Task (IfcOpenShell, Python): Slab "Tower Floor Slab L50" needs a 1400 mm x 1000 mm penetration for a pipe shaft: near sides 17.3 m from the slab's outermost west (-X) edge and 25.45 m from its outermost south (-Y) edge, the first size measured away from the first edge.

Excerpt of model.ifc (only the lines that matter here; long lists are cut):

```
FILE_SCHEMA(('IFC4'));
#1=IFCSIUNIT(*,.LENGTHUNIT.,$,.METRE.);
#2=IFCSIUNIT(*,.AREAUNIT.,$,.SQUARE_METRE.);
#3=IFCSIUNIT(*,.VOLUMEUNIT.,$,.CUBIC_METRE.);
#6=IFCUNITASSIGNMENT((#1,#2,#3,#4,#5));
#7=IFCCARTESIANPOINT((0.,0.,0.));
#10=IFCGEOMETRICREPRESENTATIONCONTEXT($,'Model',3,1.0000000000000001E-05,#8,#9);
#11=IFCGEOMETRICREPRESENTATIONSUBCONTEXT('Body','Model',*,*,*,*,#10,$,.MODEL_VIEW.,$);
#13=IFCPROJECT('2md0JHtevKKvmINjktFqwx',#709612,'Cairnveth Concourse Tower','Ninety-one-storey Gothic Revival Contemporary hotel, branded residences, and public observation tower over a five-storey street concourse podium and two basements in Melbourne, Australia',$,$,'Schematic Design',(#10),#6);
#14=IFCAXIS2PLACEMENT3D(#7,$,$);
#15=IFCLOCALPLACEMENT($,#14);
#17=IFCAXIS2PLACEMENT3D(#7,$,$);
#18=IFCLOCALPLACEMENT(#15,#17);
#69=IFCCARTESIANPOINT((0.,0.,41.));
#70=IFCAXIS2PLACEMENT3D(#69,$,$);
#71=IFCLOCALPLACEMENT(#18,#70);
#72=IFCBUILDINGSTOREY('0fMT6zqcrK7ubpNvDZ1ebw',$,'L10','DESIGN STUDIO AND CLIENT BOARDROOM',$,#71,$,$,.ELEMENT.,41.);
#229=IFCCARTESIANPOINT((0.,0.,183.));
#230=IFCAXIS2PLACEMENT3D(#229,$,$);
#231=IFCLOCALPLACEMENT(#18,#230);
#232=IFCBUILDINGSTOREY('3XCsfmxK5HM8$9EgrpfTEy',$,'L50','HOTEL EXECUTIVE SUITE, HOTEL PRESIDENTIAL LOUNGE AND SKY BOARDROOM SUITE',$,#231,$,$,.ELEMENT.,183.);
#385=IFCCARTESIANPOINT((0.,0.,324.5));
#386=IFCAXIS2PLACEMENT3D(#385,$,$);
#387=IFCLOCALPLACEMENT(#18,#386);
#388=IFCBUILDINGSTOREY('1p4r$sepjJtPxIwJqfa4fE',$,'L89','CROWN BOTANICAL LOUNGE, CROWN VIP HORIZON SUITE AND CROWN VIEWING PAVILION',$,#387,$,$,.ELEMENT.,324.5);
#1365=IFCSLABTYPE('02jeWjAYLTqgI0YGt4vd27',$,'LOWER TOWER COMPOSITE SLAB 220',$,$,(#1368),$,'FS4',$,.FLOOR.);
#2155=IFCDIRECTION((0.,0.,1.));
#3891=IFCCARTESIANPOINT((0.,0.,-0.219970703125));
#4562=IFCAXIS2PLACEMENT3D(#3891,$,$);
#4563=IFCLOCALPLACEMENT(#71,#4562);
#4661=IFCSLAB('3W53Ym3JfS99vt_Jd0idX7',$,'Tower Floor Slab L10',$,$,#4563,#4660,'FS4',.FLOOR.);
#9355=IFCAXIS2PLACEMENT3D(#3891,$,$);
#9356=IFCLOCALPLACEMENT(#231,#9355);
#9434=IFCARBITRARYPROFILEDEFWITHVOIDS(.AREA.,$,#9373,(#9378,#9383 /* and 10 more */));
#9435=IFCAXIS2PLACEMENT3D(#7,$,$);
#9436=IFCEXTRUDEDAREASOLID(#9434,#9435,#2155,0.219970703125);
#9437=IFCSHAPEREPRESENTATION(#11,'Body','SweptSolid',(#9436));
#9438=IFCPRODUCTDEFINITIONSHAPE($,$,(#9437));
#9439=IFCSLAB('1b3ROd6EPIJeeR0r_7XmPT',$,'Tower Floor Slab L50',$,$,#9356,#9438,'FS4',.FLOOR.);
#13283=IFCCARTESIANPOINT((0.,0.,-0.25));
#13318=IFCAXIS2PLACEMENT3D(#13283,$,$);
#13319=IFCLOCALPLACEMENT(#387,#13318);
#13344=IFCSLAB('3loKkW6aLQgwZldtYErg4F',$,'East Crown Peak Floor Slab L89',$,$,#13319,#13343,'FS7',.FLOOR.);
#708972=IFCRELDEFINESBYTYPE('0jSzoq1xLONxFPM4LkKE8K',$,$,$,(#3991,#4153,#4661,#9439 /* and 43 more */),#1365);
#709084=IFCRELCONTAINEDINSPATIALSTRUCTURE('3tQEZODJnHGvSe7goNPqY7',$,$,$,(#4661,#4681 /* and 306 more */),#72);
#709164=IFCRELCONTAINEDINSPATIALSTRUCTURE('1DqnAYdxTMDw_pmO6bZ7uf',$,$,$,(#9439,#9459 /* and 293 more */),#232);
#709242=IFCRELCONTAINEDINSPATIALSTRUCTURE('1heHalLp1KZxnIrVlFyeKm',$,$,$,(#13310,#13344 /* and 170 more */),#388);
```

```python
import numpy as np
import ifcopenshell
import ifcopenshell.api.feature
import ifcopenshell.api.geometry
import ifcopenshell.api.root
import ifcopenshell.geom
import ifcopenshell.util.placement
import ifcopenshell.util.representation
import ifcopenshell.util.shape
import ifcopenshell.util.unit

model = ifcopenshell.open("model.ifc")
unit_scale = ifcopenshell.util.unit.calculate_unit_scale(model)
settings = ifcopenshell.geom.settings()


def volume(element):
    """Net volume in cubic metres, openings subtracted."""
    shape = ifcopenshell.geom.create_shape(settings, element)
    return ifcopenshell.util.shape.get_volume(shape.geometry)


slab = model.by_guid("1b3ROd6EPIJeeR0r_7XmPT")
before = volume(slab)

# Extent in the slab's own axes, in metres. The edges named are its -X and -Y sides.
slab_shape = ifcopenshell.geom.create_shape(settings, slab)
vertices = ifcopenshell.util.shape.get_vertices(slab_shape.geometry)
x_min, y_min, bottom = vertices.min(axis=0)
top = vertices[:, 2].max()

opening = ifcopenshell.api.root.create_entity(model, ifc_class="IfcOpeningElement", name="Pipe shaft opening", predefined_type="OPENING")
context = ifcopenshell.util.representation.get_context(model, "Model", "Body", "MODEL_VIEW")
width, depth = 1.4, 1
outline = [(0.0, 0.0), (width, 0.0), (width, depth), (0.0, depth), (0.0, 0.0)]
# Overshoot both faces by 50 mm so the cut is clean.
shape = ifcopenshell.api.geometry.add_slab_representation(
    model, context=context, depth=top - bottom + 0.1, polyline=outline
)
ifcopenshell.api.geometry.assign_representation(model, product=opening, representation=shape)

matrix = ifcopenshell.util.placement.get_local_placement(slab.ObjectPlacement)
matrix[:, 3] = matrix @ np.append(np.array([x_min + 17.3, y_min + 25.45, bottom - 0.05]) / unit_scale, 1.0)
ifcopenshell.api.geometry.edit_object_placement(model, product=opening, matrix=matrix, is_si=False)
ifcopenshell.api.feature.add_feature(model, feature=opening, element=slab)

after = volume(slab)

print(f"slab volume {before:.3f} -> {after:.3f} m3")

model.write("model_updated.ifc")
```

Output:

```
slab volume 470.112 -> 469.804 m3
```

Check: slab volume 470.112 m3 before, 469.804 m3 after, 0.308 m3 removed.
